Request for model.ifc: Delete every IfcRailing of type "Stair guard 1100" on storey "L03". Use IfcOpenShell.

First a look at what the model holds.

```python
import ifcopenshell
import ifcopenshell.util.element

model = ifcopenshell.open("model.ifc")
print(model.schema)
storey = next(s for s in model.by_type("IfcBuildingStorey") if s.Name == "L03")
railings = [e for e in ifcopenshell.util.element.get_decomposition(storey) if e.is_a("IfcRailing")]
seen = {}
for e in railings:
    element_type = ifcopenshell.util.element.get_type(e)
    name = element_type.Name if element_type not in (None, e) else None
    seen[name] = seen.get(name, 0) + 1
for name, count in sorted(seen.items(), key=str):
    print(count, "x", name)
```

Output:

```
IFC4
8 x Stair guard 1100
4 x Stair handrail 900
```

```python
import ifcopenshell
import ifcopenshell.api.root
import ifcopenshell.util.element

model = ifcopenshell.open("model.ifc")

storey = next(s for s in model.by_type("IfcBuildingStorey") if s.Name == "L03")
railings = [e for e in ifcopenshell.util.element.get_decomposition(storey) if e.is_a("IfcRailing")]
targets = [e for e in railings if (t := ifcopenshell.util.element.get_type(e)) not in (None, e) and t.Name == "Stair guard 1100"]

for e in targets:
    ifcopenshell.api.root.remove_product(model, product=e)
print(len(targets), "removed")

model.write("model_rev.ifc")
```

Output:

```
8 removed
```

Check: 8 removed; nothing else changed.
